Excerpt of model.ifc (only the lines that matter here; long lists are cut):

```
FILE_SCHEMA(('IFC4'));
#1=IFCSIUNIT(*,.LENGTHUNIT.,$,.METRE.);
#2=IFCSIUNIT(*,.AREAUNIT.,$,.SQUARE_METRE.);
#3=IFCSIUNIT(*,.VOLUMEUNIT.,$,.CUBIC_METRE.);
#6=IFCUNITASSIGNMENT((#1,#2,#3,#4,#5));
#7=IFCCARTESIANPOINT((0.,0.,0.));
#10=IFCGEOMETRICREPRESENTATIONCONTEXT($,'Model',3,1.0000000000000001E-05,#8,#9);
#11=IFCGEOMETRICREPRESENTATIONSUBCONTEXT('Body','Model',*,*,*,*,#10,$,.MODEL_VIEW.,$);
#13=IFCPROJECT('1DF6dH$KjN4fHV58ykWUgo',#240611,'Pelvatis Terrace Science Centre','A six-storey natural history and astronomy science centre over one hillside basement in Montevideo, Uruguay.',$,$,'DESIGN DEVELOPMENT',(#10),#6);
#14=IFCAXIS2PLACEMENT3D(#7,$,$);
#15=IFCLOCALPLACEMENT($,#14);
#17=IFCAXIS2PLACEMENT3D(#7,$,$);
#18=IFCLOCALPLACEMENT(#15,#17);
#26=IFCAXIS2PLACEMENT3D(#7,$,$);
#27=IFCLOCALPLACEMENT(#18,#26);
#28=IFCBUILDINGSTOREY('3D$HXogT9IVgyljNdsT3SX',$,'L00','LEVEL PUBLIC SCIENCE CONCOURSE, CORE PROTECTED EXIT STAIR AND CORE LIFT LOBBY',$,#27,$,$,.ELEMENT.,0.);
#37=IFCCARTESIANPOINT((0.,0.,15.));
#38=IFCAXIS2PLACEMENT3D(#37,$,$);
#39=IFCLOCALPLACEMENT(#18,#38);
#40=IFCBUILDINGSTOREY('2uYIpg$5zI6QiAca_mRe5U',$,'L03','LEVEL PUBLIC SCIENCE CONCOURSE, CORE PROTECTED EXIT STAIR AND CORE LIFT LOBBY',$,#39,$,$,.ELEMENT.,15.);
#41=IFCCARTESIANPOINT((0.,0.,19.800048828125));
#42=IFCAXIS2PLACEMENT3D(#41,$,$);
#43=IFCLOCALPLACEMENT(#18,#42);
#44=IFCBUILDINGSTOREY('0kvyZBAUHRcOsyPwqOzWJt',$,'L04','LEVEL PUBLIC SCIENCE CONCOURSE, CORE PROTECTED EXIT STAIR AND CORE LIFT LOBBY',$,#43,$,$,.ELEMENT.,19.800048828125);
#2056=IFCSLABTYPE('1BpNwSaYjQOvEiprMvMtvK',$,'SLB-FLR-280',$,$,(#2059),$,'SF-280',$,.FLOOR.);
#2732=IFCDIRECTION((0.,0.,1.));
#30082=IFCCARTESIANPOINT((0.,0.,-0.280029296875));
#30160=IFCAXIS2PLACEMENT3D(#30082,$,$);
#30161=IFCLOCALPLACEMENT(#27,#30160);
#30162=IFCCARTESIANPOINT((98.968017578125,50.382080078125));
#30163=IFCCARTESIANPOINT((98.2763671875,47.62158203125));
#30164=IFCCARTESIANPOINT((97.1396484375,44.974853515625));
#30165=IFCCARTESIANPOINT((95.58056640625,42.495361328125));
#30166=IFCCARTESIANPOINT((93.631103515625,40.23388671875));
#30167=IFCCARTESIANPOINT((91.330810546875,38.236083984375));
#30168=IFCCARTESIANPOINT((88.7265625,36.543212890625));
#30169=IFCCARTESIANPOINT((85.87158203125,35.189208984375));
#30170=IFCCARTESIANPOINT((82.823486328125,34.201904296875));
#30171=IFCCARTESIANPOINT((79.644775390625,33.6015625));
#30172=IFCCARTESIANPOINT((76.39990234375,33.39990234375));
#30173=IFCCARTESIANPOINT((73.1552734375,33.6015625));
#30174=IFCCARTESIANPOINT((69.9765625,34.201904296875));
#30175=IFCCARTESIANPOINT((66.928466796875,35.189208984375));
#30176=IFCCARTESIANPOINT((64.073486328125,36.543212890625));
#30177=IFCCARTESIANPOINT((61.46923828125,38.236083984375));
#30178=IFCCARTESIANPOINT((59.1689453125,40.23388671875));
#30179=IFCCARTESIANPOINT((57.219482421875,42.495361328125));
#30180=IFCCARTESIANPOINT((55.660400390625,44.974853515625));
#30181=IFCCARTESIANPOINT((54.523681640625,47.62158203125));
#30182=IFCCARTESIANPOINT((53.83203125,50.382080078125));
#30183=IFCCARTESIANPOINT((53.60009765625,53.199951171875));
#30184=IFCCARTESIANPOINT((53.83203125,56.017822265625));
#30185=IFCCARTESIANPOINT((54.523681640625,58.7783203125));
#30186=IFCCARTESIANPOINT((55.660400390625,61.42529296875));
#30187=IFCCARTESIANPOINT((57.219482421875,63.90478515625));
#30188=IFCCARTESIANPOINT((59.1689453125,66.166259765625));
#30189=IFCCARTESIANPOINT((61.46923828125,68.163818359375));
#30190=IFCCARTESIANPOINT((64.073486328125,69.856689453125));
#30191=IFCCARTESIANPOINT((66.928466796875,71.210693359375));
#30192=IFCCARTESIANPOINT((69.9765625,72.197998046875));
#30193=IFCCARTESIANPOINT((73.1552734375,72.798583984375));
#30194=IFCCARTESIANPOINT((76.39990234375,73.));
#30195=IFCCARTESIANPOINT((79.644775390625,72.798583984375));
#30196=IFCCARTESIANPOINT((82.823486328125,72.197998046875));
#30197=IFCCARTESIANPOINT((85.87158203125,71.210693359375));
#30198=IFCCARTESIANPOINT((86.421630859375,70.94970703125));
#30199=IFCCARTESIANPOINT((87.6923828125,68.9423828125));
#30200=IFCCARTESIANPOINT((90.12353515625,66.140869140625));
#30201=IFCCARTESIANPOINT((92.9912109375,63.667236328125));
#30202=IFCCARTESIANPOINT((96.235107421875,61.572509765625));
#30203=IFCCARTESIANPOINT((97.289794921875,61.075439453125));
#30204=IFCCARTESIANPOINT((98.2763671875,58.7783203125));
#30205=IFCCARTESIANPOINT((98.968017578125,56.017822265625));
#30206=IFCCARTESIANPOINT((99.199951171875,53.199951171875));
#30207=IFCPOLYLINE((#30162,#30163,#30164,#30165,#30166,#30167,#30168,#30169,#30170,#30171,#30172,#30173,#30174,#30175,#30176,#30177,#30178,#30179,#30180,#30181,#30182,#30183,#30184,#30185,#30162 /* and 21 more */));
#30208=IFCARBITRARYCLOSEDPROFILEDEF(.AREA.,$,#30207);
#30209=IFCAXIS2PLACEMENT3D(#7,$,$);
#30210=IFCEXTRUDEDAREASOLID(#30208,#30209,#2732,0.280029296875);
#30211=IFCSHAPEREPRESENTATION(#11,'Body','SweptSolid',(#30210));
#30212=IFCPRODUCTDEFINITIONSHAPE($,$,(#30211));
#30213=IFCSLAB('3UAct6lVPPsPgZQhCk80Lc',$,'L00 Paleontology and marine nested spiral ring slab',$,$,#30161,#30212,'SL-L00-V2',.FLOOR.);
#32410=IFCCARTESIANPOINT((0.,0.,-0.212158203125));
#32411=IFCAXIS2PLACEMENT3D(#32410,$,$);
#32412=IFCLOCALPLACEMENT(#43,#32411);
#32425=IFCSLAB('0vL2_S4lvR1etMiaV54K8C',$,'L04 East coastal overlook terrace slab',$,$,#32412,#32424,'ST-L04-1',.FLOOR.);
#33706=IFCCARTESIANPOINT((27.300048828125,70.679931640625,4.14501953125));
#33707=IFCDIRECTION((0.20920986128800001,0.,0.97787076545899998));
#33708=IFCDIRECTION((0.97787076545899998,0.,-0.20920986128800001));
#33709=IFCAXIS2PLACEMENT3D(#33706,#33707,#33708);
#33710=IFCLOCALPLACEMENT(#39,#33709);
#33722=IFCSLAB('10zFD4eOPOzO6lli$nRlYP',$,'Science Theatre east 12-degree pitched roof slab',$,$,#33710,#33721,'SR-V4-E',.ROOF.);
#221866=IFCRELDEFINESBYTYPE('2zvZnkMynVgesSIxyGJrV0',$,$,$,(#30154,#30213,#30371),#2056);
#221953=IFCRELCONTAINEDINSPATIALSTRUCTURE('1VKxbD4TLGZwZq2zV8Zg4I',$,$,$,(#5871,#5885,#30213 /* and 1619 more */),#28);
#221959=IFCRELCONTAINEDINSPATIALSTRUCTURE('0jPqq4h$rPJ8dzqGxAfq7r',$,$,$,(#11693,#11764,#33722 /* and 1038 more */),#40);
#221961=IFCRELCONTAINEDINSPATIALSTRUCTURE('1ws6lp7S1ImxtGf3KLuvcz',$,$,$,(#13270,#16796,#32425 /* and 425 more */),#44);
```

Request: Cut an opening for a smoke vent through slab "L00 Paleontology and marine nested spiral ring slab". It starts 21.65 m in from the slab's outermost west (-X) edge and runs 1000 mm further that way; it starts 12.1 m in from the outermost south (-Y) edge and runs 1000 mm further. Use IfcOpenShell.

```python
import numpy as np
import ifcopenshell
import ifcopenshell.api.feature
import ifcopenshell.api.geometry
import ifcopenshell.api.root
import ifcopenshell.geom
import ifcopenshell.util.placement
import ifcopenshell.util.representation
import ifcopenshell.util.shape
import ifcopenshell.util.unit

model = ifcopenshell.open("model.ifc")
unit_scale = ifcopenshell.util.unit.calculate_unit_scale(model)
settings = ifcopenshell.geom.settings()


def volume(element):
    """Net volume in cubic metres, openings subtracted."""
    shape = ifcopenshell.geom.create_shape(settings, element)
    return ifcopenshell.util.shape.get_volume(shape.geometry)


slab = model.by_guid("3UAct6lVPPsPgZQhCk80Lc")
before = volume(slab)

# Extent in the slab's own axes, in metres. The edges named are its -X and -Y sides.
slab_shape = ifcopenshell.geom.create_shape(settings, slab)
vertices = ifcopenshell.util.shape.get_vertices(slab_shape.geometry)
x_min, y_min, bottom = vertices.min(axis=0)
top = vertices[:, 2].max()

opening = ifcopenshell.api.root.create_entity(model, ifc_class="IfcOpeningElement", name="Smoke vent opening", predefined_type="OPENING")
context = ifcopenshell.util.representation.get_context(model, "Model", "Body", "MODEL_VIEW")
width, depth = 1, 1
outline = [(0.0, 0.0), (width, 0.0), (width, depth), (0.0, depth), (0.0, 0.0)]
# Overshoot both faces by 50 mm so the cut is clean.
shape = ifcopenshell.api.geometry.add_slab_representation(
    model, context=context, depth=top - bottom + 0.1, polyline=outline
)
ifcopenshell.api.geometry.assign_representation(model, product=opening, representation=shape)

matrix = ifcopenshell.util.placement.get_local_placement(slab.ObjectPlacement)
matrix[:, 3] = matrix @ np.append(np.array([x_min + 21.65, y_min + 12.1, bottom - 0.05]) / unit_scale, 1.0)
ifcopenshell.api.geometry.edit_object_placement(model, product=opening, matrix=matrix, is_si=False)
ifcopenshell.api.feature.add_feature(model, feature=opening, element=slab)

after = volume(slab)

print(f"slab volume {before:.3f} -> {after:.3f} m3")

model.write("model_v2.ifc")
```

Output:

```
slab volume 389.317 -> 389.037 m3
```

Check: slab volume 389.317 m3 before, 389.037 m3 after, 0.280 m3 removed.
